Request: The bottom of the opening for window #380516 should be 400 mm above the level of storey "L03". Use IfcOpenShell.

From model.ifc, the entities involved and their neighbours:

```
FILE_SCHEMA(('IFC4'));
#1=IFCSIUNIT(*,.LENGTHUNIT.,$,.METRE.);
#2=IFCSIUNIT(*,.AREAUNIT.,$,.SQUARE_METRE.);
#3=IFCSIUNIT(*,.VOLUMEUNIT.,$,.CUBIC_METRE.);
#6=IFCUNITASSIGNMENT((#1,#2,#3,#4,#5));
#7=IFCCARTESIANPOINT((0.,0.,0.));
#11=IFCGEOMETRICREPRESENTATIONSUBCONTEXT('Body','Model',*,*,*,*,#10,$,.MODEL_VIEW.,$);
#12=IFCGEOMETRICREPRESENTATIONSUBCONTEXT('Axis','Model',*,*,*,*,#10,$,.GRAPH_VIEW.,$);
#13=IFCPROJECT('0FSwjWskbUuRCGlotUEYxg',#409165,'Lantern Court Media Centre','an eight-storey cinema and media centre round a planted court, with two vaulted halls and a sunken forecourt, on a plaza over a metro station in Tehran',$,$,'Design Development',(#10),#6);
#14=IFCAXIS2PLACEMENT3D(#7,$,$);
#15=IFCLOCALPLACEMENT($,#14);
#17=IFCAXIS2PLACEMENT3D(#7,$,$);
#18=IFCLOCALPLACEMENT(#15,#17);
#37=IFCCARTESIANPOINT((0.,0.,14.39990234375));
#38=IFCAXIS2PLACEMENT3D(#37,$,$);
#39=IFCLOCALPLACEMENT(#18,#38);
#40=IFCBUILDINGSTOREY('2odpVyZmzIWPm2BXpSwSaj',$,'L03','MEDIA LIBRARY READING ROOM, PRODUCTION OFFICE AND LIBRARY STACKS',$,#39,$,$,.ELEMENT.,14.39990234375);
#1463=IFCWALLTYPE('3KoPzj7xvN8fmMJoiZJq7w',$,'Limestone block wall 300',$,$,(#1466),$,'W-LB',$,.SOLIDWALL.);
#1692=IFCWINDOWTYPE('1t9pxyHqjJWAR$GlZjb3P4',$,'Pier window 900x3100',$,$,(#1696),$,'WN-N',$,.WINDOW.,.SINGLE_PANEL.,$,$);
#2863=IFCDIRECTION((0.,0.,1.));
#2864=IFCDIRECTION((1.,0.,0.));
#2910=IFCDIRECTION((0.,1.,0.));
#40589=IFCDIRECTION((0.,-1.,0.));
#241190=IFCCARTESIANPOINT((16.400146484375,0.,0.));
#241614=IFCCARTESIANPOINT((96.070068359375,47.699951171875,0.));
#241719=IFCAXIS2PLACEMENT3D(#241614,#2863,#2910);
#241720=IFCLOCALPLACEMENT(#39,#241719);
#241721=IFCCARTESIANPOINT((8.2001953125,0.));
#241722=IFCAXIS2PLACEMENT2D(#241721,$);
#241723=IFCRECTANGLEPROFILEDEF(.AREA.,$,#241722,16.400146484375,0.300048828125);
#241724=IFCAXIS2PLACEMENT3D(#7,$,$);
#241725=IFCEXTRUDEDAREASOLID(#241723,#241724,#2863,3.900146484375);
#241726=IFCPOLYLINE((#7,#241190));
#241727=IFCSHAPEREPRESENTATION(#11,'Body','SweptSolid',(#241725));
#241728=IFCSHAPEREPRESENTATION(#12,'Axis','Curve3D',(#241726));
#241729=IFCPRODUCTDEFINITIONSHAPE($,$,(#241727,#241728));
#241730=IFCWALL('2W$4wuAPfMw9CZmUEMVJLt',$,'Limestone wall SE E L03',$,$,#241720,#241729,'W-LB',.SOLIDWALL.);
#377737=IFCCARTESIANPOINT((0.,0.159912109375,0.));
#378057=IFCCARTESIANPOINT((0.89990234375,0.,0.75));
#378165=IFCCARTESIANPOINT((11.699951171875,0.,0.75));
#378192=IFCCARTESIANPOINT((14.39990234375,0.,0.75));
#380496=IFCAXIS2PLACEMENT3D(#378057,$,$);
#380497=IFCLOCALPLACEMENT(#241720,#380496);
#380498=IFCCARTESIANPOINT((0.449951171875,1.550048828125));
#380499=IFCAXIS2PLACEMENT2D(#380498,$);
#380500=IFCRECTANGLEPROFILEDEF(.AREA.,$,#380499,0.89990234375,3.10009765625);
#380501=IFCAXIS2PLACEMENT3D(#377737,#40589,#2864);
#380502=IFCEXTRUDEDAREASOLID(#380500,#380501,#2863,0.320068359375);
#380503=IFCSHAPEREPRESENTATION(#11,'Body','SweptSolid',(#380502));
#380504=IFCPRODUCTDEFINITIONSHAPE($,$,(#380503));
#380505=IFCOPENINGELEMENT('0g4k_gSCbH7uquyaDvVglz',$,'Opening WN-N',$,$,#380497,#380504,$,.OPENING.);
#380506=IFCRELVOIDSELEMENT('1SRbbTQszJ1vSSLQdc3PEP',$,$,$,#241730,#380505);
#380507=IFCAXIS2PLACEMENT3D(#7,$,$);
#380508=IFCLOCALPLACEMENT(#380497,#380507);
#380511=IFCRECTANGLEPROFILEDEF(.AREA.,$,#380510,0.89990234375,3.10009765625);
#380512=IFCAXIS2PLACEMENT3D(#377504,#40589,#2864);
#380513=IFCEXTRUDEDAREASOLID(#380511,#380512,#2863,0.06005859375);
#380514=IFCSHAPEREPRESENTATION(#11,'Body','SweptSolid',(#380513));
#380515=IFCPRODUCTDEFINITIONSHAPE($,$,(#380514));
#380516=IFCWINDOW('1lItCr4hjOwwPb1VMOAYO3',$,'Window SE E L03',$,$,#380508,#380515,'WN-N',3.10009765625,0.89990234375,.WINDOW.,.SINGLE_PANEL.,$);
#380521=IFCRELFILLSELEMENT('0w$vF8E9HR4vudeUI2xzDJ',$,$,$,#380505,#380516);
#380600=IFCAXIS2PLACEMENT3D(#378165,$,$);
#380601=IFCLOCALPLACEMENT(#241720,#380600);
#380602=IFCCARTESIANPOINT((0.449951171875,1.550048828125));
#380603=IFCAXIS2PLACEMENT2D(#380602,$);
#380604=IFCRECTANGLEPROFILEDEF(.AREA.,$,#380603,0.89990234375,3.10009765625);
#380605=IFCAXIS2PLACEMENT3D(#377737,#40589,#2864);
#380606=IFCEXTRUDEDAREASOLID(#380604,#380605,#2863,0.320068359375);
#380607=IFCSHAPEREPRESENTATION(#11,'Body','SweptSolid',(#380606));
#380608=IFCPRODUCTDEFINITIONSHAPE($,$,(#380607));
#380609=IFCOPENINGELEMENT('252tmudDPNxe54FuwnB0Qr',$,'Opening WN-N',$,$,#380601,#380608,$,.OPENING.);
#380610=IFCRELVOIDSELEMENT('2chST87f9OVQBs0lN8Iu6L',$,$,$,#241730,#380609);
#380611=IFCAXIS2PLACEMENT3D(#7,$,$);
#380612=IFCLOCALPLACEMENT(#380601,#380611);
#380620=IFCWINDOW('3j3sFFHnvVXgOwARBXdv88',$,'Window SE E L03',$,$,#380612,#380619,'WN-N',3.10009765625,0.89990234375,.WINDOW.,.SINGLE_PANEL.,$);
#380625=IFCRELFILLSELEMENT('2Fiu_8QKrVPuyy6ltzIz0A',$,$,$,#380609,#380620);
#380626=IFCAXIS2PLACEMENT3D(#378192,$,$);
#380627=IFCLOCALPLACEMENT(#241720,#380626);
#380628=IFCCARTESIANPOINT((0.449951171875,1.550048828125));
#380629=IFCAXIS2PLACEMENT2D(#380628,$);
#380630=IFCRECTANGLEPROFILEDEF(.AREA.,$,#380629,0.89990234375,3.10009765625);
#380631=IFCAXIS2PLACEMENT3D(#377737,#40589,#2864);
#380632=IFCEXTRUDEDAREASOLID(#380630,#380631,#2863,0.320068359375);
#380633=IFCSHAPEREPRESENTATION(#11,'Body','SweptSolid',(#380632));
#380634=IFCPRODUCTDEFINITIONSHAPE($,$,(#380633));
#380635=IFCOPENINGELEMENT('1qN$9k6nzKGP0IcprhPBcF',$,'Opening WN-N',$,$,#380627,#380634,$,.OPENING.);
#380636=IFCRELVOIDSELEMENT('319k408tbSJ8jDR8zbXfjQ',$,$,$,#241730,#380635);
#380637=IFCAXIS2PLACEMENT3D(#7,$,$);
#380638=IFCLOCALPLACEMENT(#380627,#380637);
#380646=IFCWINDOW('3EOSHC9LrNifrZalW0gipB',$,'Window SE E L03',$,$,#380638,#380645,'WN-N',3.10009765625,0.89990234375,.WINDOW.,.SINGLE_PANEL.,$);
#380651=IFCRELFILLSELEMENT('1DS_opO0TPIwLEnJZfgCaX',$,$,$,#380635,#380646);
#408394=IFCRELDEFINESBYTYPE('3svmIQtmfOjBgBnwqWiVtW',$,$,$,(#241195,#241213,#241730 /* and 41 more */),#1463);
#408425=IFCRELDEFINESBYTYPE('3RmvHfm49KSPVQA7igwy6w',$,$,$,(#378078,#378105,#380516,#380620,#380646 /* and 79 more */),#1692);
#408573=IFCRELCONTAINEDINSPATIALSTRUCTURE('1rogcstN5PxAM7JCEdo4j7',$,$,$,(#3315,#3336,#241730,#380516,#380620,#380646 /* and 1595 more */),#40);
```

```python
import numpy as np
import ifcopenshell
import ifcopenshell.api.geometry
import ifcopenshell.geom
import ifcopenshell.util.element
import ifcopenshell.util.placement
import ifcopenshell.util.shape
import ifcopenshell.util.unit

model = ifcopenshell.open("model.ifc")
unit_scale = ifcopenshell.util.unit.calculate_unit_scale(model)

window = model.by_guid("1lItCr4hjOwwPb1VMOAYO3")
opening = window.FillsVoids[0].RelatingOpeningElement
storey = ifcopenshell.util.element.get_container(window, ifc_class="IfcBuildingStorey")
level = ifcopenshell.util.placement.get_local_placement(storey.ObjectPlacement)[2, 3]

# The opening's origin need not be at the sill, so measure its lowest point.
shape = ifcopenshell.geom.create_shape(ifcopenshell.geom.settings(), opening)
bottom = ifcopenshell.util.shape.get_shape_bottom_elevation(shape, shape.geometry) / unit_scale
dz = level + 0.4 / unit_scale - bottom

shift = np.array([0.0, 0.0, dz])
# The window is placed relative to its opening, so it follows when the opening moves.
matrix = ifcopenshell.util.placement.get_local_placement(opening.ObjectPlacement)
matrix[:3, 3] += shift
ifcopenshell.api.geometry.edit_object_placement(
    model, product=opening, matrix=matrix, is_si=False, should_transform_children=True
)

print(f"moved by {dz * unit_scale:+.3f} m")

model.write("model_updated.ifc")
```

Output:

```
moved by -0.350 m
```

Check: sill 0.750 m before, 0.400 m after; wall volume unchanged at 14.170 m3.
